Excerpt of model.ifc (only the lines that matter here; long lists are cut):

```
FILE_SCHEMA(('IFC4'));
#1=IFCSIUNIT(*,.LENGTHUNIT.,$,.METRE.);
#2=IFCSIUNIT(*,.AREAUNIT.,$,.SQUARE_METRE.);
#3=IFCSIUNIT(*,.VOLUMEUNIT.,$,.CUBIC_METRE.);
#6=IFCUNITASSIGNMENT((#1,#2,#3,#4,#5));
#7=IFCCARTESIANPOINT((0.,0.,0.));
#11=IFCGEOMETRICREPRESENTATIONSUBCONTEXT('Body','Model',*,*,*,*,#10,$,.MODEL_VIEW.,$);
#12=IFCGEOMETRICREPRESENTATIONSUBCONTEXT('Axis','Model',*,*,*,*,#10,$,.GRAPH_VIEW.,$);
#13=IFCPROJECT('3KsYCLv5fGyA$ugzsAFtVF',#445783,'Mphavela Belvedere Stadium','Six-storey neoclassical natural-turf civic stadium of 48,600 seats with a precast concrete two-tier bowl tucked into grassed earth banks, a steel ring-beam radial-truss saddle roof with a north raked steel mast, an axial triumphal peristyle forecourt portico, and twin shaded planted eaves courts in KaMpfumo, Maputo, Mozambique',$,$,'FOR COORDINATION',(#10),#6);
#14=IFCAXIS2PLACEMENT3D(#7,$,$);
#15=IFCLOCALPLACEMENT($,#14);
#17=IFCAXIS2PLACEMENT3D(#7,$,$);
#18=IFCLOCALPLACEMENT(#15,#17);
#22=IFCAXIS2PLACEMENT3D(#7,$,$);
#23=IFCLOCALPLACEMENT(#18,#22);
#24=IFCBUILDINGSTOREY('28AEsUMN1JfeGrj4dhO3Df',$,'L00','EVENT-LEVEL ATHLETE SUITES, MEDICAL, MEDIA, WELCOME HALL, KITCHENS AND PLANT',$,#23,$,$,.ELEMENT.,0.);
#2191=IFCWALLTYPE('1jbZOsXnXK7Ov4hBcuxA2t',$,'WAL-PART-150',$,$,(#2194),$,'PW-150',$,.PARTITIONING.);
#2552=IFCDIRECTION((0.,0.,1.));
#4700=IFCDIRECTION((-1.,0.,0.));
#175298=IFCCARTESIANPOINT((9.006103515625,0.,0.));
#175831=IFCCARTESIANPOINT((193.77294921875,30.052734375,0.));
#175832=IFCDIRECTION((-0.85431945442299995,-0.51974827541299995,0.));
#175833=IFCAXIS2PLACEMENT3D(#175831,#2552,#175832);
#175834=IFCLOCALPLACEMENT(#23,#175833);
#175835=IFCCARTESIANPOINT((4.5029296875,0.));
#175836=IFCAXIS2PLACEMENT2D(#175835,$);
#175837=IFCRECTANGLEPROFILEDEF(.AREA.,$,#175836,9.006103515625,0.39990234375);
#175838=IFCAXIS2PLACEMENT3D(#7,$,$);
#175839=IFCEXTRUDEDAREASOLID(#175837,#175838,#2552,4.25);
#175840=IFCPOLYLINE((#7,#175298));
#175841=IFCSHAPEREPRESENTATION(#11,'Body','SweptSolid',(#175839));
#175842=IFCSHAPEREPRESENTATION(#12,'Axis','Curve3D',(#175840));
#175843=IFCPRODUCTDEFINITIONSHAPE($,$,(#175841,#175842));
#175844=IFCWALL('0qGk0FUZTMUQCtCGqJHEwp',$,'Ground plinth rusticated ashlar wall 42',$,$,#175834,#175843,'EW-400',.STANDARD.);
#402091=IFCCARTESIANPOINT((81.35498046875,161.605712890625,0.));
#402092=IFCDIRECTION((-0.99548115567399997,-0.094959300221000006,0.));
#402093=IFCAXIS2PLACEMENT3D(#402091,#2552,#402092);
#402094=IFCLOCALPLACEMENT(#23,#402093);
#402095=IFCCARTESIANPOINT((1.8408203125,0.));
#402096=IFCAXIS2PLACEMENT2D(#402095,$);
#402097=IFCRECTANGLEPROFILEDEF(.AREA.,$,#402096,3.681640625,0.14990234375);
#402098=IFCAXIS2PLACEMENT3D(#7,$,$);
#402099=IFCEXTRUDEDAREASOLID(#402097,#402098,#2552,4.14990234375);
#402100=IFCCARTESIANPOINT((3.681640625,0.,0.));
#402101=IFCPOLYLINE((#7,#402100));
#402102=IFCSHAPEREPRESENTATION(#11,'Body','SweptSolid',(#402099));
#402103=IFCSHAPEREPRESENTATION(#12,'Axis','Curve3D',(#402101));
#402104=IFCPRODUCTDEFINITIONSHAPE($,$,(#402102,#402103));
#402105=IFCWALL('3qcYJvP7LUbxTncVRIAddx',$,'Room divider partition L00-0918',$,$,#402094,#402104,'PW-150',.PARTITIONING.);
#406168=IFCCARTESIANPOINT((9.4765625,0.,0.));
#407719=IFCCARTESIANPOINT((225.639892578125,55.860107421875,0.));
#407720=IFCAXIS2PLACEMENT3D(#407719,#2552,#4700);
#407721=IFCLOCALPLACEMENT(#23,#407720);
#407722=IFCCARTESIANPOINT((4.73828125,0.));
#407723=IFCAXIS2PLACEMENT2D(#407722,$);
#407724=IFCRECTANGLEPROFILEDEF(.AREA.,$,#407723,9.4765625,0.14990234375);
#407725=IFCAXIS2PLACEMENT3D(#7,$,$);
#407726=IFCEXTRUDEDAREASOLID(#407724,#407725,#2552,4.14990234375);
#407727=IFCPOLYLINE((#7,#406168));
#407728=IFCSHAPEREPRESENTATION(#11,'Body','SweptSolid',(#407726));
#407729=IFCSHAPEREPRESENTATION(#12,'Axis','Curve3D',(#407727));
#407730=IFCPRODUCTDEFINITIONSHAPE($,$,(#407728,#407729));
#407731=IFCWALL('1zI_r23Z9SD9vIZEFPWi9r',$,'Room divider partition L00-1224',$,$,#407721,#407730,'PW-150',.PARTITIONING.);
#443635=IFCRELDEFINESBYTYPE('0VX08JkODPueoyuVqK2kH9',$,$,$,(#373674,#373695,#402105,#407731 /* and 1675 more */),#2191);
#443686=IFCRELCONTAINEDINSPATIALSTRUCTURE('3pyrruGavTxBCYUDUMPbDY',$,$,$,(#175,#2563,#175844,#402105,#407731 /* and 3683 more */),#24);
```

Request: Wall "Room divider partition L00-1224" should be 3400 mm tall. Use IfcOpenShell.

```python
import ifcopenshell
import ifcopenshell.geom
import ifcopenshell.util.representation
import ifcopenshell.util.shape

model = ifcopenshell.open("model.ifc")
settings = ifcopenshell.geom.settings()


def volume(element):
    """Net volume in cubic metres, openings subtracted."""
    shape = ifcopenshell.geom.create_shape(settings, element)
    return ifcopenshell.util.shape.get_volume(shape.geometry)


wall = model.by_guid("1zI_r23Z9SD9vIZEFPWi9r")
before = volume(wall)

body = ifcopenshell.util.representation.get_representation(wall, "Model", "Body")
solid = body.Items[0]
old_height = solid.Depth
solid.Depth = 3.4
after = volume(wall)

print(f"height {old_height:g} -> {solid.Depth:g}, volume {before:.3f} -> {after:.3f} m3")

model.write("model_rev.ifc")
```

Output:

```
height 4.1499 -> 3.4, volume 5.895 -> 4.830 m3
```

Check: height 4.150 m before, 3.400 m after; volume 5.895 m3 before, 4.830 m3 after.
